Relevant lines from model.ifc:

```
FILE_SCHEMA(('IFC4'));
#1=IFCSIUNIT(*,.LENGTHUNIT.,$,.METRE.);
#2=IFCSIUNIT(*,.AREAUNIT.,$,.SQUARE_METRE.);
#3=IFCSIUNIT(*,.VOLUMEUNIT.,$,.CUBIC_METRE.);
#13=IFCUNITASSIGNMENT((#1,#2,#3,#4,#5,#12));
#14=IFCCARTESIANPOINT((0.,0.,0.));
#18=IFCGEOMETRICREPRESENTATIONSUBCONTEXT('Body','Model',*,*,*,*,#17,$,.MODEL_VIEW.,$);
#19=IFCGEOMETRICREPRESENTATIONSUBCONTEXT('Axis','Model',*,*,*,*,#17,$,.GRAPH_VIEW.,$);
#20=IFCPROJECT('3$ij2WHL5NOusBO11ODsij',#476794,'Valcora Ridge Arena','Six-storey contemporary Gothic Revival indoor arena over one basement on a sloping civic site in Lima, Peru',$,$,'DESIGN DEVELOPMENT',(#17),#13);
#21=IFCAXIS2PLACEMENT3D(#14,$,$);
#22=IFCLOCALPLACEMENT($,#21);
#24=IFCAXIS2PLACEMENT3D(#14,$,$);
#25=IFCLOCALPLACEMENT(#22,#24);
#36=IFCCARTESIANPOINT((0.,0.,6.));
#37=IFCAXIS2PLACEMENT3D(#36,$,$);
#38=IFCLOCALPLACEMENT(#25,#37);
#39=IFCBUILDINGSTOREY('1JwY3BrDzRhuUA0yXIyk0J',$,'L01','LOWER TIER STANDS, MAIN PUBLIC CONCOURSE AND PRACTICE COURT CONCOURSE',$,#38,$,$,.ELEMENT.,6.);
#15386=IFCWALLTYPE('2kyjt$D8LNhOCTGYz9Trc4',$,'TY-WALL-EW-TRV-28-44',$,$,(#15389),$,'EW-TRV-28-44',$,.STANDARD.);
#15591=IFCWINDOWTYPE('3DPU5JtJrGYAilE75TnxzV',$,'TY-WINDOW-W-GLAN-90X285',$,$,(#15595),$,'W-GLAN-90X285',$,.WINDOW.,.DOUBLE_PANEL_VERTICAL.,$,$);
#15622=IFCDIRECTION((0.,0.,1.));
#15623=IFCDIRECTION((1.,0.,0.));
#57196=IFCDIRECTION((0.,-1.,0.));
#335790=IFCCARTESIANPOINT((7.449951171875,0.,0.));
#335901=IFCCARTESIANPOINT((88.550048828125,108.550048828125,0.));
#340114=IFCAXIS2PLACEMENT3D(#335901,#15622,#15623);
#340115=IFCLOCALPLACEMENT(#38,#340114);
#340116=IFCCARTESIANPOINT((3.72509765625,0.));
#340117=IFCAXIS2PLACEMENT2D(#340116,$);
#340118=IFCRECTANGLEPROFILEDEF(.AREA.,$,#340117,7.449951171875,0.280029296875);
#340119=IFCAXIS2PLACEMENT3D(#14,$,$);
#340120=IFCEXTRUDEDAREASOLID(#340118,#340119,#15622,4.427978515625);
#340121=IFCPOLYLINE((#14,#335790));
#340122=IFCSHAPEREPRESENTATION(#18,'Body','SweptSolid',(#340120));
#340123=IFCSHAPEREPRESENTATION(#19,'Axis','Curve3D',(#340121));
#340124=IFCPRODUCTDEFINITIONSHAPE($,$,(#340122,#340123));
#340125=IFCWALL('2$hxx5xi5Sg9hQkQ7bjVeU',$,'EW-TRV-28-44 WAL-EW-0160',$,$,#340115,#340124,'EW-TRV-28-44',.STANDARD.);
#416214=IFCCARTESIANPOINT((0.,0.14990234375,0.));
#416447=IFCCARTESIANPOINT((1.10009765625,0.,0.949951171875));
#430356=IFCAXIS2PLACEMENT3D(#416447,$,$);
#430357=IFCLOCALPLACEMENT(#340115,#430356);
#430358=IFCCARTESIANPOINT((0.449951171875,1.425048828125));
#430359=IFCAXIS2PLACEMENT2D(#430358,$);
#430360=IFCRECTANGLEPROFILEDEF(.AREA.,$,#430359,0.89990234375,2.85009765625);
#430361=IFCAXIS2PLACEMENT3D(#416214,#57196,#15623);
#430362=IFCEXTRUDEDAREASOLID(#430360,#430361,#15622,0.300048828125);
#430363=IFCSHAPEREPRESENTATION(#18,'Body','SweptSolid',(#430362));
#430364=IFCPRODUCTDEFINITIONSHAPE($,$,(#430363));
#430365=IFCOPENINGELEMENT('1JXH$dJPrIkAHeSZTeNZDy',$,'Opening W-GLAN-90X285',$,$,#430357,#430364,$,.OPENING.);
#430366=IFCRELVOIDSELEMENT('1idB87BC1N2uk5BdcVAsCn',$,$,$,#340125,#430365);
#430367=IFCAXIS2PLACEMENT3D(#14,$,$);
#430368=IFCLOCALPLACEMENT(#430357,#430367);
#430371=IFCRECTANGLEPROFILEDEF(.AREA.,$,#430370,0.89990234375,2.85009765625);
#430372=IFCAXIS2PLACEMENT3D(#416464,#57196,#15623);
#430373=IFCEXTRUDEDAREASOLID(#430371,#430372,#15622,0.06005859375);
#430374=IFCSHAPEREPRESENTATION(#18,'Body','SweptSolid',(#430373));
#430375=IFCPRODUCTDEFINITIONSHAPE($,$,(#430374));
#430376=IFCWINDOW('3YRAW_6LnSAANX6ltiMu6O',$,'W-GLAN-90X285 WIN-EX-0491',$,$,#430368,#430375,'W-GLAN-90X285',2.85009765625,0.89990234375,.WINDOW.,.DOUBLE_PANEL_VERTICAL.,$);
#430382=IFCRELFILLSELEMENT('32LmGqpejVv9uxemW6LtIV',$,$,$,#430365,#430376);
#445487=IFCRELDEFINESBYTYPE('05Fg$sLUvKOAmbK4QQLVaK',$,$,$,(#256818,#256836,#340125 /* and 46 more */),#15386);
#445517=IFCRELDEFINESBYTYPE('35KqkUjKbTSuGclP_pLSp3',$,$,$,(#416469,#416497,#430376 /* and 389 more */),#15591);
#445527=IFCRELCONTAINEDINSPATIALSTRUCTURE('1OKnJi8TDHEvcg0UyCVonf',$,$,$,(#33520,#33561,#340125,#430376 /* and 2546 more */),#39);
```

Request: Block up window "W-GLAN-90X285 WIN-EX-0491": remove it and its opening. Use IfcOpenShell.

```python
import ifcopenshell
import ifcopenshell.api.feature
import ifcopenshell.api.root
import ifcopenshell.geom
import ifcopenshell.util.shape

model = ifcopenshell.open("model.ifc")
settings = ifcopenshell.geom.settings()


def volume(element):
    """Net volume in cubic metres, openings subtracted."""
    shape = ifcopenshell.geom.create_shape(settings, element)
    return ifcopenshell.util.shape.get_volume(shape.geometry)


window = model.by_guid("3YRAW_6LnSAANX6ltiMu6O")
opening = window.FillsVoids[0].RelatingOpeningElement
wall = opening.VoidsElements[0].RelatingBuildingElement
before = volume(wall)

ifcopenshell.api.root.remove_product(model, product=window)
ifcopenshell.api.feature.remove_feature(model, feature=opening)

after = volume(wall)

print(f"wall volume {before:.3f} -> {after:.3f} m3")

model.write("model_edited.ifc")
```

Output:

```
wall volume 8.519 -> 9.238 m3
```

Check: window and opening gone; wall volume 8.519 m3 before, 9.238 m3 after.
